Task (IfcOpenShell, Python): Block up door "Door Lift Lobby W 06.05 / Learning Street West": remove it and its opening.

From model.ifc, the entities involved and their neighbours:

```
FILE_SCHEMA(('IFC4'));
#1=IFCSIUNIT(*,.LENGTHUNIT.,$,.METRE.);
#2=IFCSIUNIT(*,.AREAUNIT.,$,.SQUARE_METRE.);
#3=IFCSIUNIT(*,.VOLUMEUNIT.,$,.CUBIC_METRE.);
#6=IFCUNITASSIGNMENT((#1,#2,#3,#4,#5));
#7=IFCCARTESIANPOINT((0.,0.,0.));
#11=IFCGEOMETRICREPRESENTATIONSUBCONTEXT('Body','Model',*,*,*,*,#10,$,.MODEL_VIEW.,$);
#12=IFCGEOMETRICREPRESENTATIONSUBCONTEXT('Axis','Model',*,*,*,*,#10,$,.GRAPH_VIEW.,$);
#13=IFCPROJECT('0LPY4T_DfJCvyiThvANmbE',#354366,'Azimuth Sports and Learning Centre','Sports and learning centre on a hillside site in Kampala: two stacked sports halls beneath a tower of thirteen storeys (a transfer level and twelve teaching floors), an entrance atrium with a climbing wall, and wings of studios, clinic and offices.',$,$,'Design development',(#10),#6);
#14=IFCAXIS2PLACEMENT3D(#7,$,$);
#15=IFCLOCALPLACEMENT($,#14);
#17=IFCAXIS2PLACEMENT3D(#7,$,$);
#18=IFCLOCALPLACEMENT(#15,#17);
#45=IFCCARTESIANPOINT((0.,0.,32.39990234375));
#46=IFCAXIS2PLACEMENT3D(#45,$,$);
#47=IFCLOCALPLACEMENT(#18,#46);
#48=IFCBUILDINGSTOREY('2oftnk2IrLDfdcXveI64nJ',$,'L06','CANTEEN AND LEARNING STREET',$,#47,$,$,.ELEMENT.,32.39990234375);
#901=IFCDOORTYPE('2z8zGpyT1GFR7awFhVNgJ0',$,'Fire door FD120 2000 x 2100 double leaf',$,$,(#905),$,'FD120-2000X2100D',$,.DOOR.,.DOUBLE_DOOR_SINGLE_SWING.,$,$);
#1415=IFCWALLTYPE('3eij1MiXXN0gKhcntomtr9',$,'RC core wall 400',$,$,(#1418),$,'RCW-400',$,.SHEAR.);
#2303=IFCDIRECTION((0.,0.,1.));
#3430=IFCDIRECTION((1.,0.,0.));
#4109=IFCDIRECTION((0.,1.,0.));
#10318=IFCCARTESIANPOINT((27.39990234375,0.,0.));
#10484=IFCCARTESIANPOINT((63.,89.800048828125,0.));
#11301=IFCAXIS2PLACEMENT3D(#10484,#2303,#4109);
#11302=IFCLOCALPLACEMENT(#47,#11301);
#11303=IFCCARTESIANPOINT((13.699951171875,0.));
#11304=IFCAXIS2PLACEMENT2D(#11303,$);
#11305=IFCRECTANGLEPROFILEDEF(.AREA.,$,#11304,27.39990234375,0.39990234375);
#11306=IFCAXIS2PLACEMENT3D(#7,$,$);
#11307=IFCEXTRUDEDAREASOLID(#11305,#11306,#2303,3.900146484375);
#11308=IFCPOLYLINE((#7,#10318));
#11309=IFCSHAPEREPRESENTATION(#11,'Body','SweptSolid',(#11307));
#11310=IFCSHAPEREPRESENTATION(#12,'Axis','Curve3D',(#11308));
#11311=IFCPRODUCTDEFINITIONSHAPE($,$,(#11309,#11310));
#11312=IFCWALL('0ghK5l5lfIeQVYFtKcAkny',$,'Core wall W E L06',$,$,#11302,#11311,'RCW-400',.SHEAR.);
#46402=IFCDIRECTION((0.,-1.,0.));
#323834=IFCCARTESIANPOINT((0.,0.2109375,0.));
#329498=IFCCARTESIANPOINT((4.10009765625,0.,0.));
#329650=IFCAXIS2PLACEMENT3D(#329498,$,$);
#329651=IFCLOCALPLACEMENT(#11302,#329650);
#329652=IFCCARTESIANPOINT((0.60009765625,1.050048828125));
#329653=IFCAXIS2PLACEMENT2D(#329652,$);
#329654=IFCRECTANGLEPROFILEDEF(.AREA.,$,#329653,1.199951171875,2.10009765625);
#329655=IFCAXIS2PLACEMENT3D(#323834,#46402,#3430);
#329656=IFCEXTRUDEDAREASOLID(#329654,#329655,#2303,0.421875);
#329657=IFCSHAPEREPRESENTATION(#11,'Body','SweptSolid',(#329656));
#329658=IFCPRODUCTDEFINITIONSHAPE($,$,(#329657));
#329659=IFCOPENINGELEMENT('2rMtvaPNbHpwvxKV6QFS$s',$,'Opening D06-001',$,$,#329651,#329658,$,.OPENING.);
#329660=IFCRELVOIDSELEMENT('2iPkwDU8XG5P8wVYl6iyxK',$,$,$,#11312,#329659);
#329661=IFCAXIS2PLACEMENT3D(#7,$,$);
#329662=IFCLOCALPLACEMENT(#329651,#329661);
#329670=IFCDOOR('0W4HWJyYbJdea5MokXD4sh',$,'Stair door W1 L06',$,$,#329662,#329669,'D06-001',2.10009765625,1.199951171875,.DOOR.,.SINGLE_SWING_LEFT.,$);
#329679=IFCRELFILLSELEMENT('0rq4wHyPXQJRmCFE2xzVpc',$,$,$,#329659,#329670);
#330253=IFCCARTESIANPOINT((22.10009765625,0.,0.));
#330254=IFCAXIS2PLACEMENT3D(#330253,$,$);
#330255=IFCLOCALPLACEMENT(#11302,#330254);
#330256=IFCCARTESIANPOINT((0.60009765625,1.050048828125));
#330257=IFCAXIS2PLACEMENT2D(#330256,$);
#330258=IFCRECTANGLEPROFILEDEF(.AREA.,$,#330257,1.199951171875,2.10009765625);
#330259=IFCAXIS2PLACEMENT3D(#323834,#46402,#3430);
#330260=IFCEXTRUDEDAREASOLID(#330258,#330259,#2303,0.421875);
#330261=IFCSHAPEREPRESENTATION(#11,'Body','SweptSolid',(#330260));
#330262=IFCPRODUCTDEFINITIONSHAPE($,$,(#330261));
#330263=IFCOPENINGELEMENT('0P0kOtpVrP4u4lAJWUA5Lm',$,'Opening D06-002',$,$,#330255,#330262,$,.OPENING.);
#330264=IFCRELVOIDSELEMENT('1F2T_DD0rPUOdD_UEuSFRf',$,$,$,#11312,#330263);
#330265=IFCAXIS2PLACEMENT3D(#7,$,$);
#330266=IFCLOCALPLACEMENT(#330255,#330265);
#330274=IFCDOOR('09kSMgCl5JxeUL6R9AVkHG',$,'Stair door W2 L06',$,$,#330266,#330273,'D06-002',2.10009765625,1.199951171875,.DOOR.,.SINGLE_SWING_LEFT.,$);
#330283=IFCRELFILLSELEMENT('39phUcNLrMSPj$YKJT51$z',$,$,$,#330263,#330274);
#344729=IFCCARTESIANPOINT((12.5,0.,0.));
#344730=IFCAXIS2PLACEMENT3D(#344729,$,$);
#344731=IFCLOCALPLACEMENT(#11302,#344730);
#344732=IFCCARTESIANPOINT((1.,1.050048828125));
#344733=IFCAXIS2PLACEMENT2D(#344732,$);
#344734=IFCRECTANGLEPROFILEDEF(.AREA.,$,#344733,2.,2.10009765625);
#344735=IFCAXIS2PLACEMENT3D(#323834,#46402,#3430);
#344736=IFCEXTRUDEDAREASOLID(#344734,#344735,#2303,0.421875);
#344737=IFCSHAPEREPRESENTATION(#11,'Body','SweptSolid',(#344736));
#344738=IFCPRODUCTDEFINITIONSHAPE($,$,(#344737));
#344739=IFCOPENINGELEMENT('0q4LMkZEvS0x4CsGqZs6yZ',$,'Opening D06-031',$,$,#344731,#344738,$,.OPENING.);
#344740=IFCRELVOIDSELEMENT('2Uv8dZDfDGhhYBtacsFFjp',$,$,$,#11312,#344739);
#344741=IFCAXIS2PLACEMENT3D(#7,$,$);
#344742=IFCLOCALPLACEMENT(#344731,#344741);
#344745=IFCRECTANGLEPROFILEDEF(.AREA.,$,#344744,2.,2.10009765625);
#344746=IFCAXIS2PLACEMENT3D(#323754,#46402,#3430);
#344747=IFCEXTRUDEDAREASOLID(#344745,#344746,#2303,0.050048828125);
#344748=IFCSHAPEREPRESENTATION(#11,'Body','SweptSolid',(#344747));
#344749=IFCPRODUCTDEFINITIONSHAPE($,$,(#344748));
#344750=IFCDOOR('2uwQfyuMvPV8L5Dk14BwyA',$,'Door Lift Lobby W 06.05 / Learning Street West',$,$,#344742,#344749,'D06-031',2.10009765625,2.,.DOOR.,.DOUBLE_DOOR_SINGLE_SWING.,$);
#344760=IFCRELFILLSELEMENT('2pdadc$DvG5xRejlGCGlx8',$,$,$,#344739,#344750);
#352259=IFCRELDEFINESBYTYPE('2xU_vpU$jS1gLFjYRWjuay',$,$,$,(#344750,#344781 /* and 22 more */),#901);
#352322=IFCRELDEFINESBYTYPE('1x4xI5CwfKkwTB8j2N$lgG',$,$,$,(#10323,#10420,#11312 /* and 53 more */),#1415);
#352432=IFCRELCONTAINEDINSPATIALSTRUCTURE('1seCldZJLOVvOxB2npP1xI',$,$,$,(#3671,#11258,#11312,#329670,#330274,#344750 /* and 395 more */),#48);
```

```python
import ifcopenshell
import ifcopenshell.api.feature
import ifcopenshell.api.root
import ifcopenshell.geom
import ifcopenshell.util.shape

model = ifcopenshell.open("model.ifc")
settings = ifcopenshell.geom.settings()


def volume(element):
    """Net volume in cubic metres, openings subtracted."""
    shape = ifcopenshell.geom.create_shape(settings, element)
    return ifcopenshell.util.shape.get_volume(shape.geometry)


door = model.by_guid("2uwQfyuMvPV8L5Dk14BwyA")
opening = door.FillsVoids[0].RelatingOpeningElement
wall = opening.VoidsElements[0].RelatingBuildingElement
before = volume(wall)

ifcopenshell.api.root.remove_product(model, product=door)
ifcopenshell.api.feature.remove_feature(model, feature=opening)

after = volume(wall)

print(f"wall volume {before:.3f} -> {after:.3f} m3")

model.write("model_edited.ifc")
```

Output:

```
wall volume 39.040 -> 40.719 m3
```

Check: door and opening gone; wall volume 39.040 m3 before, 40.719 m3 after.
